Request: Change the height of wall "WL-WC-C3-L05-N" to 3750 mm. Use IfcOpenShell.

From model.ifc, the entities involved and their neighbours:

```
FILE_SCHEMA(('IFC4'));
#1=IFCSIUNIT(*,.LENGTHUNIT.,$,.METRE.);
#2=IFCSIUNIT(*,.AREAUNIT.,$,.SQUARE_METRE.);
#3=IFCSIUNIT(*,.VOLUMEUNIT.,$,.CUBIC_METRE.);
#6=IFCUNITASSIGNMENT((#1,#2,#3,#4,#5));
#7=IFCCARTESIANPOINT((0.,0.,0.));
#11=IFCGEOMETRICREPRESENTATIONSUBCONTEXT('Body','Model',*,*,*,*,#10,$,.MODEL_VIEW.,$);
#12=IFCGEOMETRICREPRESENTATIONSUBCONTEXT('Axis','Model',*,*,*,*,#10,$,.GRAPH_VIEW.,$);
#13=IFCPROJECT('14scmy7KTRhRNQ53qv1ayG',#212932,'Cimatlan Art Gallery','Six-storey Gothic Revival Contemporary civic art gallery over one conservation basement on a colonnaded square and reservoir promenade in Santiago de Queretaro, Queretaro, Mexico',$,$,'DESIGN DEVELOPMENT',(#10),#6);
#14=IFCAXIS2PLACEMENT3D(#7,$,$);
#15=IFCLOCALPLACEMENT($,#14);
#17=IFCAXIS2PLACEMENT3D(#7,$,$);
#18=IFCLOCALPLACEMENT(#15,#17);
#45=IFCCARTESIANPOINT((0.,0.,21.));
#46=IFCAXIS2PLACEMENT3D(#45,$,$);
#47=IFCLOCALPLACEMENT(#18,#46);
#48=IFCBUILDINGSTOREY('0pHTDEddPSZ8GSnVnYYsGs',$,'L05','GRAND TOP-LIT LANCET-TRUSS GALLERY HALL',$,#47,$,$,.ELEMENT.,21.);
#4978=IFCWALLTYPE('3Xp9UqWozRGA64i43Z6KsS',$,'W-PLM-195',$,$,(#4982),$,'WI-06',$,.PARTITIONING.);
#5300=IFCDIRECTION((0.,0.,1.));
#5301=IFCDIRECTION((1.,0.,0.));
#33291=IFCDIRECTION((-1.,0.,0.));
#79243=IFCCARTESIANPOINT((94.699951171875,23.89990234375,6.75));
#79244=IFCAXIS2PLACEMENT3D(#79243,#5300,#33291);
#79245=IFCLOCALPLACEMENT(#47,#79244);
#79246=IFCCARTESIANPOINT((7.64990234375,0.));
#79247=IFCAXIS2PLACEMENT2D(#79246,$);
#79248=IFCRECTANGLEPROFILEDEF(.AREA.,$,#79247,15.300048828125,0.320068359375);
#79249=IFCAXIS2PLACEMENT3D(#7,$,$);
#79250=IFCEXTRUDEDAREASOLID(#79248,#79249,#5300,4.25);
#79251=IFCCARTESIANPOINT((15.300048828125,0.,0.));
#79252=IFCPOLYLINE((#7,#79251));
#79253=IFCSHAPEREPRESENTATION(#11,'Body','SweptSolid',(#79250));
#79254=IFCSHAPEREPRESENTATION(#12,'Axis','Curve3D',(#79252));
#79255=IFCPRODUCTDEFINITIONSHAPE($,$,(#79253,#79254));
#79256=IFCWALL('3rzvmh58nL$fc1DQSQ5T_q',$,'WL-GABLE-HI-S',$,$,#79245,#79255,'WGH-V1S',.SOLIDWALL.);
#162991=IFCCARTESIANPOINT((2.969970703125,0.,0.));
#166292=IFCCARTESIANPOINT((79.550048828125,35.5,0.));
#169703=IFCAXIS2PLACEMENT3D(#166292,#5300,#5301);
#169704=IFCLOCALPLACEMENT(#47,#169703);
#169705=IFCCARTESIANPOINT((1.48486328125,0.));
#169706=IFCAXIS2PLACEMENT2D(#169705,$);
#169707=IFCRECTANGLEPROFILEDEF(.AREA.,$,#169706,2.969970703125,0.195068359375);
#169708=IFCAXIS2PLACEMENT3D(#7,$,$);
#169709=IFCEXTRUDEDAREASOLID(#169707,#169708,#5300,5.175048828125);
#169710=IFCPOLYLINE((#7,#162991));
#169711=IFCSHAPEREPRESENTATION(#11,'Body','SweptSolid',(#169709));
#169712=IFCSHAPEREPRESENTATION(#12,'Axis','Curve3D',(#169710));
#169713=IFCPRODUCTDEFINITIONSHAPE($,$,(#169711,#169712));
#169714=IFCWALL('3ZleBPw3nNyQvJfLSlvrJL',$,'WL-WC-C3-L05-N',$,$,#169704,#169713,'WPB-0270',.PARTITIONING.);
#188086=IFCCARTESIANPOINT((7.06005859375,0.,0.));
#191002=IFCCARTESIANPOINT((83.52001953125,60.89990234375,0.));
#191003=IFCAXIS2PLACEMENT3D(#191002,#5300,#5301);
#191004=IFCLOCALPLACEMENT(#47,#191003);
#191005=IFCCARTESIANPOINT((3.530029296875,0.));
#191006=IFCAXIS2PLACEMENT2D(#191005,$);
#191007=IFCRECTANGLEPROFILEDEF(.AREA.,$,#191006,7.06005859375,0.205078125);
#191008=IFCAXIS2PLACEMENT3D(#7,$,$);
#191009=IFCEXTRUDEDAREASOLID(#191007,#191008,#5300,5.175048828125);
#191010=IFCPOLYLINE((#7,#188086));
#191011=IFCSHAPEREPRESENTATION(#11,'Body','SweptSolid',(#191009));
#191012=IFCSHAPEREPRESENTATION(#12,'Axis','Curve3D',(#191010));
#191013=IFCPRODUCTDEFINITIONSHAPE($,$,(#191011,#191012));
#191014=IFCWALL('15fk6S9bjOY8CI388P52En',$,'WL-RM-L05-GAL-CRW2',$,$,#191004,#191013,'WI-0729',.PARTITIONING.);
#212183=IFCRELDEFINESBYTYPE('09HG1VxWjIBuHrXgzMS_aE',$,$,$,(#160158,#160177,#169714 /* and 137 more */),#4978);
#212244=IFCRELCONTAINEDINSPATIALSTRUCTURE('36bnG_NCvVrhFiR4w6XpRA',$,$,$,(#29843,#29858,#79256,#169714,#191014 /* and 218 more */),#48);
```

```python
import ifcopenshell
import ifcopenshell.geom
import ifcopenshell.util.representation
import ifcopenshell.util.shape
import ifcopenshell.util.unit

model = ifcopenshell.open("model.ifc")
unit_scale = ifcopenshell.util.unit.calculate_unit_scale(model)
settings = ifcopenshell.geom.settings()


def volume(element):
    """Net volume in cubic metres, openings subtracted."""
    shape = ifcopenshell.geom.create_shape(settings, element)
    return ifcopenshell.util.shape.get_volume(shape.geometry)


wall = model.by_guid("3ZleBPw3nNyQvJfLSlvrJL")
before = volume(wall)

body = ifcopenshell.util.representation.get_representation(wall, "Model", "Body")
solid = body.Items[0]
old_height = solid.Depth
solid.Depth = 3.75 / unit_scale
after = volume(wall)

print(f"height {old_height:g} -> {solid.Depth:g}, volume {before:.3f} -> {after:.3f} m3")

model.write("model_v2.ifc")
```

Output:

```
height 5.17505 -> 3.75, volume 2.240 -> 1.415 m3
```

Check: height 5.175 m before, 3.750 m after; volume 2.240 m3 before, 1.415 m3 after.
